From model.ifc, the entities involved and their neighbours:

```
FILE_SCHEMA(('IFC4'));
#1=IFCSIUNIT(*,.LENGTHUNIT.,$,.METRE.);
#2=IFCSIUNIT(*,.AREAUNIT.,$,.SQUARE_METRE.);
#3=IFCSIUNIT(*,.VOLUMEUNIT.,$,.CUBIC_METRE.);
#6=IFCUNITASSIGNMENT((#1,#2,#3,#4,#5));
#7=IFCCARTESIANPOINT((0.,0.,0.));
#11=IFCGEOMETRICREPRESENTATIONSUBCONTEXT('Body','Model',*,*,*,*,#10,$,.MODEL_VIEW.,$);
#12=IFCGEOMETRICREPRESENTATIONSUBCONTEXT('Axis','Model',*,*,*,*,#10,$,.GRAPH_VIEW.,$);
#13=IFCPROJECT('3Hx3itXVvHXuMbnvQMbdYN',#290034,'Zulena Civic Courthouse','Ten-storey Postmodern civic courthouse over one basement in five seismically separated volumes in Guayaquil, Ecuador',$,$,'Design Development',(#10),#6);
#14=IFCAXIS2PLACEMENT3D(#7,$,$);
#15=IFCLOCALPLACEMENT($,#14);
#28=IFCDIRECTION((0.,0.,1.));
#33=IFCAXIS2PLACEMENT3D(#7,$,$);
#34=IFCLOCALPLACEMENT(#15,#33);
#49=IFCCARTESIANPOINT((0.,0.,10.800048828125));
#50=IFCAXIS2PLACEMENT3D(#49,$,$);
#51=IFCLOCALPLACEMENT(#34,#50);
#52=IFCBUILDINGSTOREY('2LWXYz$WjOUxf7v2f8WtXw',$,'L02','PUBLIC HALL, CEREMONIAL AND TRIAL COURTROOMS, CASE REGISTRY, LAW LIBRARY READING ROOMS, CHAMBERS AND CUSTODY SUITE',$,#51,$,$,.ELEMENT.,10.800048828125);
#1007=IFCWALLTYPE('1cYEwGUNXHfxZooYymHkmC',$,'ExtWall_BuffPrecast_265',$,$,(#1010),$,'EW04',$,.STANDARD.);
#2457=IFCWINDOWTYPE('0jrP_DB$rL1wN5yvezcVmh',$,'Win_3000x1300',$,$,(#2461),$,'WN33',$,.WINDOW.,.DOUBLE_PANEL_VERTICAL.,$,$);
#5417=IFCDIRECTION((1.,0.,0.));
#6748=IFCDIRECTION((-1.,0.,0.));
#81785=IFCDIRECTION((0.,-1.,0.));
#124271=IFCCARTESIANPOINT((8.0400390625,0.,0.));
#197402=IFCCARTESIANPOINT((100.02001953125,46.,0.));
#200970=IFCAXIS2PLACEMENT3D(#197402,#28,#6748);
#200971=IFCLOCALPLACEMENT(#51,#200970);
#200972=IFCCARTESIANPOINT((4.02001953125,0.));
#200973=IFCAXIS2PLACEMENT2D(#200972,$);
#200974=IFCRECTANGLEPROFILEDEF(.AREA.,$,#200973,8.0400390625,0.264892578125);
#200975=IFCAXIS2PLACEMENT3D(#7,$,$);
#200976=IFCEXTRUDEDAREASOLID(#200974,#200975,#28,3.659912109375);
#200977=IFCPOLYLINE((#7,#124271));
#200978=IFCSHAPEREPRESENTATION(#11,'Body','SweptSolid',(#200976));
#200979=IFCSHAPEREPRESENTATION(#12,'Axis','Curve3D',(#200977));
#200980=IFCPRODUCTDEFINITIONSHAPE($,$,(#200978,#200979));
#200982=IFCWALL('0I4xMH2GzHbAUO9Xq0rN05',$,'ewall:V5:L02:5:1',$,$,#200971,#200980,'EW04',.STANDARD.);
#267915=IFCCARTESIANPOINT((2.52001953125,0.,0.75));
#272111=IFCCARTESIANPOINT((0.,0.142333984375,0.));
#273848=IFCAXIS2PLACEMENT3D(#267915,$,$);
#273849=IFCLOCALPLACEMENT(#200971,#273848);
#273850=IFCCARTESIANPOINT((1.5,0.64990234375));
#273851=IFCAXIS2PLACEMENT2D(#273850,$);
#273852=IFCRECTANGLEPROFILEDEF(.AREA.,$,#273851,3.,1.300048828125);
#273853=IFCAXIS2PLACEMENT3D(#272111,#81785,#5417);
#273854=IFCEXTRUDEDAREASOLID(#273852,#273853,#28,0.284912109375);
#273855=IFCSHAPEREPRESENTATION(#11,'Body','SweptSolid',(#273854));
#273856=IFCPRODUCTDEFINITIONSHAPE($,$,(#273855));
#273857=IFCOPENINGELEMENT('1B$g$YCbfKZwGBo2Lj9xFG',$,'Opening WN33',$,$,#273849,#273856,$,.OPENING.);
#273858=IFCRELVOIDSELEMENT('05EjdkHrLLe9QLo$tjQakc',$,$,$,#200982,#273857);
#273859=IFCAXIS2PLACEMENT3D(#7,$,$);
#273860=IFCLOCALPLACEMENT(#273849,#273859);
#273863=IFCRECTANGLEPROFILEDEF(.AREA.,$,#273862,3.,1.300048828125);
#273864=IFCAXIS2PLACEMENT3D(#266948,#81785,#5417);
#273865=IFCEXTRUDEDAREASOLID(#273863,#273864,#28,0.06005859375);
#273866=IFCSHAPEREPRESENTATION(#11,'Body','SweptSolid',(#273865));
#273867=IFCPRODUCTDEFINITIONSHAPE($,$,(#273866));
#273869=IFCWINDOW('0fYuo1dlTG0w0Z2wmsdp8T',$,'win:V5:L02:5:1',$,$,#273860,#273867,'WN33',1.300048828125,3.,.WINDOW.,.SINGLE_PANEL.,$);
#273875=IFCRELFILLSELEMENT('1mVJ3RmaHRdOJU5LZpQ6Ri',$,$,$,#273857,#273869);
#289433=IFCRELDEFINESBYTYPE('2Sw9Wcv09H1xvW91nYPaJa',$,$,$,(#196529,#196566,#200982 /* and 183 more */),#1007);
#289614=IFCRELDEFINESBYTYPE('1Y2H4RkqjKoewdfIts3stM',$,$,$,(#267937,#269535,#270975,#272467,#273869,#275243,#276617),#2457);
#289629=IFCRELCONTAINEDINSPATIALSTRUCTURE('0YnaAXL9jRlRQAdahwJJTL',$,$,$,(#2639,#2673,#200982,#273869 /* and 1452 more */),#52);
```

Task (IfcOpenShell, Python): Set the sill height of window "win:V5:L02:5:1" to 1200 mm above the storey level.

```python
import numpy as np
import ifcopenshell
import ifcopenshell.api.geometry
import ifcopenshell.geom
import ifcopenshell.util.element
import ifcopenshell.util.placement
import ifcopenshell.util.shape
import ifcopenshell.util.unit

model = ifcopenshell.open("model.ifc")
unit_scale = ifcopenshell.util.unit.calculate_unit_scale(model)

window = model.by_guid("0fYuo1dlTG0w0Z2wmsdp8T")
opening = window.FillsVoids[0].RelatingOpeningElement
storey = ifcopenshell.util.element.get_container(window, ifc_class="IfcBuildingStorey")
level = ifcopenshell.util.placement.get_local_placement(storey.ObjectPlacement)[2, 3]

# The opening's origin need not be at the sill, so measure its lowest point.
shape = ifcopenshell.geom.create_shape(ifcopenshell.geom.settings(), opening)
bottom = ifcopenshell.util.shape.get_shape_bottom_elevation(shape, shape.geometry) / unit_scale
dz = level + 1.2 / unit_scale - bottom

shift = np.array([0.0, 0.0, dz])
# The window is placed relative to its opening, so it follows when the opening moves.
matrix = ifcopenshell.util.placement.get_local_placement(opening.ObjectPlacement)
matrix[:3, 3] += shift
ifcopenshell.api.geometry.edit_object_placement(
    model, product=opening, matrix=matrix, is_si=False, should_transform_children=True
)

print(f"moved by {dz * unit_scale:+.3f} m")

model.write("model_edited.ifc")
```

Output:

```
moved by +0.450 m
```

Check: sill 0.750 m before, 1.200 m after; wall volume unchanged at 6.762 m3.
